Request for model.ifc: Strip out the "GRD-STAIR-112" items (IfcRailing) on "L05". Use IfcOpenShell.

First a look at what the model holds.

```python
import ifcopenshell
import ifcopenshell.util.element

model = ifcopenshell.open("model.ifc")
print(model.schema)
storey = next(s for s in model.by_type("IfcBuildingStorey") if s.Name == "L05")
railings = [e for e in ifcopenshell.util.element.get_decomposition(storey) if e.is_a("IfcRailing")]
seen = {}
for e in railings:
    element_type = ifcopenshell.util.element.get_type(e)
    name = element_type.Name if element_type not in (None, e) else None
    seen[name] = seen.get(name, 0) + 1
for name, count in sorted(seen.items(), key=str):
    print(count, "x", name)
```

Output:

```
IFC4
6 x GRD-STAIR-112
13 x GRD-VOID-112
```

```python
import ifcopenshell
import ifcopenshell.api.root
import ifcopenshell.util.element

model = ifcopenshell.open("model.ifc")

storey = next(s for s in model.by_type("IfcBuildingStorey") if s.Name == "L05")
railings = [e for e in ifcopenshell.util.element.get_decomposition(storey) if e.is_a("IfcRailing")]
targets = [e for e in railings if (t := ifcopenshell.util.element.get_type(e)) not in (None, e) and t.Name == "GRD-STAIR-112"]

for e in targets:
    ifcopenshell.api.root.remove_product(model, product=e)
print(len(targets), "removed")

model.write("model_edited.ifc")
```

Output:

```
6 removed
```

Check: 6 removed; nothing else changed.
